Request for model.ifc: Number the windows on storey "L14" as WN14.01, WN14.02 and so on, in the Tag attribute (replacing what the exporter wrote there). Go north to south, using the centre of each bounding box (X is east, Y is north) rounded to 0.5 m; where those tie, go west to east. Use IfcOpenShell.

First a look at what the model holds.

```python
import ifcopenshell
import ifcopenshell.util.element
import ifcopenshell.util.placement

model = ifcopenshell.open("model.ifc")
print(model.schema)
storey = next(s for s in model.by_type("IfcBuildingStorey") if s.Name == "L14")
windows = [e for e in ifcopenshell.util.element.get_decomposition(storey) if e.is_a("IfcWindow")]
for e in sorted(windows, key=lambda e: e.id()):
    origin = ifcopenshell.util.placement.get_local_placement(e.ObjectPlacement)[:3, 3]
    print(e.id(), e.Tag, e.Name, origin.round(2) + 0.0, sep=" | ")
```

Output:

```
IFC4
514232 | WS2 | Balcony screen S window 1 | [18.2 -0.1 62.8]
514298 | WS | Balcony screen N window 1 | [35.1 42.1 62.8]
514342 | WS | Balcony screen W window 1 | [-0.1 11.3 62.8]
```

```python
import ifcopenshell
import ifcopenshell.geom
import ifcopenshell.util.element
import ifcopenshell.util.shape

model = ifcopenshell.open("model.ifc")
settings = ifcopenshell.geom.settings()
settings.set("use-world-coords", True)


def centre(element):
    shape = ifcopenshell.geom.create_shape(settings, element)
    return ifcopenshell.util.shape.get_bbox_centroid(shape.geometry)


storey = next(s for s in model.by_type("IfcBuildingStorey") if s.Name == "L14")
windows = [e for e in ifcopenshell.util.element.get_decomposition(storey) if e.is_a("IfcWindow")]

# Insertion points can sit at a corner or the storey origin, so sort by the geometry (in metres).
centres = {e: centre(e) for e in windows}
windows.sort(key=lambda e: (-round(centres[e][1] / 0.5), centres[e][0]))

for i, e in enumerate(windows, start=1):
    number = f"WN14.{i:02d}"
    e.Tag = number
    print(e.id(), number)

model.write("model_updated.ifc")
```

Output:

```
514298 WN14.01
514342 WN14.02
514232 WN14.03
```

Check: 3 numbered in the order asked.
